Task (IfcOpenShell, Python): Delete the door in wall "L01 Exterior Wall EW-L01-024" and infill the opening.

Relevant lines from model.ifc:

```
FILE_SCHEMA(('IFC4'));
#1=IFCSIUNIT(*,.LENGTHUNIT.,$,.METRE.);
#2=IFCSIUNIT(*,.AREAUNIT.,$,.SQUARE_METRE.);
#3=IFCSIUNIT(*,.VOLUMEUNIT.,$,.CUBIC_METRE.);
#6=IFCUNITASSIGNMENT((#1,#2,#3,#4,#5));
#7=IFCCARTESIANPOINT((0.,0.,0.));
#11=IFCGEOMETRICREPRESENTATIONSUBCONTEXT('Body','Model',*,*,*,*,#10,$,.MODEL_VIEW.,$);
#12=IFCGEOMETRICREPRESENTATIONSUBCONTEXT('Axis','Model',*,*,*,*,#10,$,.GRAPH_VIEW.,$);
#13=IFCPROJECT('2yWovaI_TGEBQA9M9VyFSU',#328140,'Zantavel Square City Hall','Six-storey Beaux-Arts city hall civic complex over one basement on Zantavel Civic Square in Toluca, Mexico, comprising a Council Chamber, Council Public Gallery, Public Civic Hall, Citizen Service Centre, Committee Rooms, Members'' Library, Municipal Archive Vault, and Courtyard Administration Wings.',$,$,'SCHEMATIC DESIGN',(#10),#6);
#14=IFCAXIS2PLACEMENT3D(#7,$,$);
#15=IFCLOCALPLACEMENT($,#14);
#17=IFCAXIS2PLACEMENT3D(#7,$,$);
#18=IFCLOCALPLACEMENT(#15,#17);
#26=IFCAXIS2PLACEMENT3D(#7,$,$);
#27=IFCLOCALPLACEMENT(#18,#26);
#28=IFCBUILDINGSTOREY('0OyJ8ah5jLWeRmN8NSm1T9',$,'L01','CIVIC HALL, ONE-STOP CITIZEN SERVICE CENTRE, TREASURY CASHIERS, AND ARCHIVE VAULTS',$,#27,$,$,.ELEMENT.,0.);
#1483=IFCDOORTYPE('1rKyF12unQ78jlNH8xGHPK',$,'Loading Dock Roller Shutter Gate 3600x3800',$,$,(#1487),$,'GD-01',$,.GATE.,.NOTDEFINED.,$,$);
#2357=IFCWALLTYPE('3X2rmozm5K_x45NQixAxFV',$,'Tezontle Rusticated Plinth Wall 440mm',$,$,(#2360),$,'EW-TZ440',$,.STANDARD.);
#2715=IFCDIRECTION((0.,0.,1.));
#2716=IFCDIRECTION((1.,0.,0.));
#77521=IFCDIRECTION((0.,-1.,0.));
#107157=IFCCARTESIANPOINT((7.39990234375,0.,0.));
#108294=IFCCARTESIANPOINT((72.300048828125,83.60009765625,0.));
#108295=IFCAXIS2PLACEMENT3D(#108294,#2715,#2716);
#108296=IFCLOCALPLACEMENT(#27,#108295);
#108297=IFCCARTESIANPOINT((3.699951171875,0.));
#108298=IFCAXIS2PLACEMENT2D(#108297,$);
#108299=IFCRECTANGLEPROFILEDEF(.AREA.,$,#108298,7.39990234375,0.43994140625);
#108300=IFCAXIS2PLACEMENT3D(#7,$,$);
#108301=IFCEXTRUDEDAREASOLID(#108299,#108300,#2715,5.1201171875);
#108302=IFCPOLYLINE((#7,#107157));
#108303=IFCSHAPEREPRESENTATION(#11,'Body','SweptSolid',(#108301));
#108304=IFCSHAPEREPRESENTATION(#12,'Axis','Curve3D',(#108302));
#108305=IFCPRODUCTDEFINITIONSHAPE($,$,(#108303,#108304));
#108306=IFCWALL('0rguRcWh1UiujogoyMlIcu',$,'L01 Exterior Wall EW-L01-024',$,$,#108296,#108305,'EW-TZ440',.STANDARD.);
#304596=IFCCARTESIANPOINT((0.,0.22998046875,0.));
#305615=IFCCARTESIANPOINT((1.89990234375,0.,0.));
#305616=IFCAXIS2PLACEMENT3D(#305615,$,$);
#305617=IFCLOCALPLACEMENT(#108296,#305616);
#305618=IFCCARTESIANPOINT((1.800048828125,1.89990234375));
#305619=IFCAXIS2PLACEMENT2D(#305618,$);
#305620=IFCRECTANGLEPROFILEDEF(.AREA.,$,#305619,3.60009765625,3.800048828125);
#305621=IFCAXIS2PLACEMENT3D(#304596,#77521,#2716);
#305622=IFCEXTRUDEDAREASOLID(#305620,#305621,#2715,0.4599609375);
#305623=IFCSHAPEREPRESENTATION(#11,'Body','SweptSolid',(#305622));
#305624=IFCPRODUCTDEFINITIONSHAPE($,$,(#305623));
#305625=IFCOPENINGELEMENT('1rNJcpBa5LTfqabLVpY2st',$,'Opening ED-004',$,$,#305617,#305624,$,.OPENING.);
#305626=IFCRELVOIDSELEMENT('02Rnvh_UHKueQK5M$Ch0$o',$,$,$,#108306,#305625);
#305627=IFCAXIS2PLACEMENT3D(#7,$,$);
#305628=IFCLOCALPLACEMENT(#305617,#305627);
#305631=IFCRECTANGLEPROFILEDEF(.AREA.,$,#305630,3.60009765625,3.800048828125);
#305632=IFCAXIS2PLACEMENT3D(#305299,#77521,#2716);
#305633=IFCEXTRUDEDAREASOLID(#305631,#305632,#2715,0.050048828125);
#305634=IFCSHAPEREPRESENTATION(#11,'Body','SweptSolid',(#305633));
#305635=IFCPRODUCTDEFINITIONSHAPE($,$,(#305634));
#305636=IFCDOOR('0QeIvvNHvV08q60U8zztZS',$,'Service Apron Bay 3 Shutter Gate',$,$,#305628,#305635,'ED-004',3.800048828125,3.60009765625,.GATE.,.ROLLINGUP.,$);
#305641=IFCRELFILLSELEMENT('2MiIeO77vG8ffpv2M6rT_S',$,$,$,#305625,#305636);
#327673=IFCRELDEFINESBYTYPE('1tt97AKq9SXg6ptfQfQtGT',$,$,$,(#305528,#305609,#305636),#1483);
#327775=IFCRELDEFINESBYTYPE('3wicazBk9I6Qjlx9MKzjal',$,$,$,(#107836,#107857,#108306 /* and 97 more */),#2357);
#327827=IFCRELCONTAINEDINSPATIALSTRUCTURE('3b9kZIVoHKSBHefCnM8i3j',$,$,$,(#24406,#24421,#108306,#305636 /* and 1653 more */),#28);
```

```python
import ifcopenshell
import ifcopenshell.api.feature
import ifcopenshell.api.root
import ifcopenshell.geom
import ifcopenshell.util.shape

model = ifcopenshell.open("model.ifc")
settings = ifcopenshell.geom.settings()


def volume(element):
    """Net volume in cubic metres, openings subtracted."""
    shape = ifcopenshell.geom.create_shape(settings, element)
    return ifcopenshell.util.shape.get_volume(shape.geometry)


door = model.by_guid("0QeIvvNHvV08q60U8zztZS")
opening = door.FillsVoids[0].RelatingOpeningElement
wall = opening.VoidsElements[0].RelatingBuildingElement
before = volume(wall)

ifcopenshell.api.root.remove_product(model, product=door)
ifcopenshell.api.feature.remove_feature(model, feature=opening)

after = volume(wall)

print(f"wall volume {before:.3f} -> {after:.3f} m3")

model.write("model_edited.ifc")
```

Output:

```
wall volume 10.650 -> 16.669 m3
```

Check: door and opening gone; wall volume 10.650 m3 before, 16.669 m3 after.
